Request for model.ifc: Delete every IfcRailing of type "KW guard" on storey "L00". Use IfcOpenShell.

First a look at what the model holds.

```python
import ifcopenshell
import ifcopenshell.util.element

model = ifcopenshell.open("model.ifc")
print(model.schema)
storey = next(s for s in model.by_type("IfcBuildingStorey") if s.Name == "L00")
railings = [e for e in ifcopenshell.util.element.get_decomposition(storey) if e.is_a("IfcRailing")]
seen = {}
for e in railings:
    element_type = ifcopenshell.util.element.get_type(e)
    name = element_type.Name if element_type not in (None, e) else None
    seen[name] = seen.get(name, 0) + 1
for name, count in sorted(seen.items(), key=str):
    print(count, "x", name)
```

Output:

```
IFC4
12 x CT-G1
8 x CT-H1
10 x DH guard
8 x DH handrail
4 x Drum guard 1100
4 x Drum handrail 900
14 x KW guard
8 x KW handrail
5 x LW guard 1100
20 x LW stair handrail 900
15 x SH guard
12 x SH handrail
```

```python
import ifcopenshell
import ifcopenshell.api.root
import ifcopenshell.util.element

model = ifcopenshell.open("model.ifc")

storey = next(s for s in model.by_type("IfcBuildingStorey") if s.Name == "L00")
railings = [e for e in ifcopenshell.util.element.get_decomposition(storey) if e.is_a("IfcRailing")]
targets = [e for e in railings if (t := ifcopenshell.util.element.get_type(e)) not in (None, e) and t.Name == "KW guard"]

for e in targets:
    ifcopenshell.api.root.remove_product(model, product=e)
print(len(targets), "removed")

model.write("model_edited.ifc")
```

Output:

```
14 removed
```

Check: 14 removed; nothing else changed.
